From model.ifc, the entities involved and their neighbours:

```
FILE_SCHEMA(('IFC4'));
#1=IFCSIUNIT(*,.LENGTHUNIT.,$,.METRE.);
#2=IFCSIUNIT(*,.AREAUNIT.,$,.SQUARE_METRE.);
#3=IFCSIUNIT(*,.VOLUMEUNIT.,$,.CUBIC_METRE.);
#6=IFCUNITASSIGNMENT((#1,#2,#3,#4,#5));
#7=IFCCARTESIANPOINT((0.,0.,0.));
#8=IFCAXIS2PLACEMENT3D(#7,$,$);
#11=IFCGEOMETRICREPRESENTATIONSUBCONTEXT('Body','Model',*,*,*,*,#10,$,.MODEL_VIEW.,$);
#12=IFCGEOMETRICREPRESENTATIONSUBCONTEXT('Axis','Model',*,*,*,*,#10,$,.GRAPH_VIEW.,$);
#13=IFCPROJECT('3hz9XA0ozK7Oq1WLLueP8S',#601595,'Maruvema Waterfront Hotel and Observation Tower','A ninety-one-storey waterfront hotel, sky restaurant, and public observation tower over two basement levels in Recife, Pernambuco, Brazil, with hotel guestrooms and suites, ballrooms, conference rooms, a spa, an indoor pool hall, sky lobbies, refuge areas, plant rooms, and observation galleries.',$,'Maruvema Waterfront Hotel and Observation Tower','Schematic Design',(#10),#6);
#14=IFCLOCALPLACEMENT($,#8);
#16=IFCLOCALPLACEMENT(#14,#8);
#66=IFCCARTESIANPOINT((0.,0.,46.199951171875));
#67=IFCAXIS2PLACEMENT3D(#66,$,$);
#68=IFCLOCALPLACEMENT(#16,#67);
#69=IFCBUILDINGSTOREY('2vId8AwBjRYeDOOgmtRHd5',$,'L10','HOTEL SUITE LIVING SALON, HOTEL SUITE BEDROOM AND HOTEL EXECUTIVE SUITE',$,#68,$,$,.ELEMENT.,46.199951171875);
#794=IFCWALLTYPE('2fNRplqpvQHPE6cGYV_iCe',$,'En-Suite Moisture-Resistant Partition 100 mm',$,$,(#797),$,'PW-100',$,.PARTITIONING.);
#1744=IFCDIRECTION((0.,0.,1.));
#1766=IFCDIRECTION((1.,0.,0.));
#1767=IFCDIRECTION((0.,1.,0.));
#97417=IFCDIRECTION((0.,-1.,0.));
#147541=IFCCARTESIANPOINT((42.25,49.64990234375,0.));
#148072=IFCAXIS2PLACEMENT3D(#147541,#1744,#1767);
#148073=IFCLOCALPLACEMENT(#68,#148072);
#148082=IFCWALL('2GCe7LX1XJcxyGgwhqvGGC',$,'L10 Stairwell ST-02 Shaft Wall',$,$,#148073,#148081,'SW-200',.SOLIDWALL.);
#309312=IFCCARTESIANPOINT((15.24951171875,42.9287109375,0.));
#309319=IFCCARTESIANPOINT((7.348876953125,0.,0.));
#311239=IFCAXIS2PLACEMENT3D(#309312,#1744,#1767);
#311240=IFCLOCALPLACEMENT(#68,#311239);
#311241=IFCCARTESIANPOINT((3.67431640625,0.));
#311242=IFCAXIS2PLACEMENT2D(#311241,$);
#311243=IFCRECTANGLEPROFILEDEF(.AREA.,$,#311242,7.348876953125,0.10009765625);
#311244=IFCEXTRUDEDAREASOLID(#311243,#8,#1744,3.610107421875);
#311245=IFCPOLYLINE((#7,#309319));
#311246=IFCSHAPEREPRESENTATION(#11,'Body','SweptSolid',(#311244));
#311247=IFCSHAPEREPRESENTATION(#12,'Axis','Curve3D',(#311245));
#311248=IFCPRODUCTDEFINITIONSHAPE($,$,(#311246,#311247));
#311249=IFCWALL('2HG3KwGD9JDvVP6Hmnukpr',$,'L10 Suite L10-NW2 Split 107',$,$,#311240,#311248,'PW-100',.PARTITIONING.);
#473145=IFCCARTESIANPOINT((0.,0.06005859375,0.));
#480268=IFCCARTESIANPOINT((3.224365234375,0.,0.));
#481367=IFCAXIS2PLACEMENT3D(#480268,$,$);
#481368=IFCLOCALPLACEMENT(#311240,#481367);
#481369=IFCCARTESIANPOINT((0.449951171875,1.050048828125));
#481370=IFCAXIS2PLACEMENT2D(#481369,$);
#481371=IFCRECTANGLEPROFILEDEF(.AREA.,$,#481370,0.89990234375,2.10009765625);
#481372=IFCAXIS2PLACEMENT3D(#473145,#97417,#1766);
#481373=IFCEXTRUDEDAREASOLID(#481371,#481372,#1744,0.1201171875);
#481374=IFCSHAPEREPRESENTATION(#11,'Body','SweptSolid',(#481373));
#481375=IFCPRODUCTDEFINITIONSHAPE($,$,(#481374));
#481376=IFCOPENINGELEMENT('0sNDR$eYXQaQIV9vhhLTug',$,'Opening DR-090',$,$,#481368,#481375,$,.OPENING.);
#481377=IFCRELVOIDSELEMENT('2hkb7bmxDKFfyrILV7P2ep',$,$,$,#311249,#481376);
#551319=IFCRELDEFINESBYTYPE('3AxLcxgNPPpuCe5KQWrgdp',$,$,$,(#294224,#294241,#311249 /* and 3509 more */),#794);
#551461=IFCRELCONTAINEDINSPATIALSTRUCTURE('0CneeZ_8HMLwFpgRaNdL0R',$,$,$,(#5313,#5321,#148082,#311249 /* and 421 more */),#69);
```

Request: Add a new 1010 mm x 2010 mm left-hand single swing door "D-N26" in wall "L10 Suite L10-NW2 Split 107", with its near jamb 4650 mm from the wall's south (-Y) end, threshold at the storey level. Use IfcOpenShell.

```python
import numpy as np
import ifcopenshell
import ifcopenshell.api.feature
import ifcopenshell.api.geometry
import ifcopenshell.api.root
import ifcopenshell.api.spatial
import ifcopenshell.geom
import ifcopenshell.util.element
import ifcopenshell.util.placement
import ifcopenshell.util.representation
import ifcopenshell.util.shape
import ifcopenshell.util.unit

model = ifcopenshell.open("model.ifc")
unit_scale = ifcopenshell.util.unit.calculate_unit_scale(model)
settings = ifcopenshell.geom.settings()


def volume(element):
    """Net volume in cubic metres, openings subtracted."""
    shape = ifcopenshell.geom.create_shape(settings, element)
    return ifcopenshell.util.shape.get_volume(shape.geometry)


wall = model.by_guid("2HG3KwGD9JDvVP6Hmnukpr")
storey = ifcopenshell.util.element.get_container(wall, ifc_class="IfcBuildingStorey")
context = ifcopenshell.util.representation.get_context(model, "Model", "Body", "MODEL_VIEW")
before = volume(wall)

width, height, from_end, sill = 1.01, 2.01, 4.65, 0.0  # metres

# The wall runs along its own X axis, and the end named is its -X end.
wall_shape = ifcopenshell.geom.create_shape(settings, wall)
x, y, z = ifcopenshell.util.shape.get_vertices(wall_shape.geometry).T
start = x.min() + from_end
face, thickness = float(y.min()), float(y.max() - y.min())
wall_matrix = ifcopenshell.util.placement.get_local_placement(wall.ObjectPlacement)
level = ifcopenshell.util.placement.get_local_placement(storey.ObjectPlacement)[2, 3]


def in_wall(x, y):
    """Placement at x, y metres in the wall's axes, at sill height."""
    matrix = wall_matrix.copy()
    matrix[:, 3] = wall_matrix @ np.array([x / unit_scale, y / unit_scale, 0.0, 1.0])
    matrix[2, 3] = level + sill / unit_scale
    return matrix


# Opening: a box that overshoots both wall faces by 50 mm.
opening = ifcopenshell.api.root.create_entity(model, ifc_class="IfcOpeningElement", predefined_type="OPENING")
box = ifcopenshell.api.geometry.add_wall_representation(
    model, context=context, length=width, height=height, thickness=thickness + 0.1
)
ifcopenshell.api.geometry.assign_representation(model, product=opening, representation=box)
ifcopenshell.api.geometry.edit_object_placement(model, product=opening, matrix=in_wall(start, face - 0.05), is_si=False)
ifcopenshell.api.feature.add_feature(model, feature=opening, element=wall)

door = ifcopenshell.api.root.create_entity(model, ifc_class="IfcDoor", name="D-N26", predefined_type="DOOR")
door.OverallWidth, door.OverallHeight = width / unit_scale, height / unit_scale
door.OperationType = "SINGLE_SWING_LEFT"
body = ifcopenshell.api.geometry.add_door_representation(
    model,
    context=context,
    overall_width=door.OverallWidth,
    overall_height=door.OverallHeight,
    operation_type="SINGLE_SWING_LEFT",
    lining_properties={"LiningDepth": thickness / unit_scale, "ThresholdDepth": thickness / unit_scale},
)
ifcopenshell.api.geometry.assign_representation(model, product=door, representation=body)
ifcopenshell.api.spatial.assign_container(model, products=[door], relating_structure=storey)
ifcopenshell.api.feature.add_filling(model, opening=opening, element=door)

# The lining spans the wall, so the door starts at the wall face.
ifcopenshell.api.geometry.edit_object_placement(model, product=door, matrix=in_wall(start, face), is_si=False)

after = volume(wall)

print(f"wall volume {before:.3f} -> {after:.3f} m3")

model.write("model-out.ifc")
```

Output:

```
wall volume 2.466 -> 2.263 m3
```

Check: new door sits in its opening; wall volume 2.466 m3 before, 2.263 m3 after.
